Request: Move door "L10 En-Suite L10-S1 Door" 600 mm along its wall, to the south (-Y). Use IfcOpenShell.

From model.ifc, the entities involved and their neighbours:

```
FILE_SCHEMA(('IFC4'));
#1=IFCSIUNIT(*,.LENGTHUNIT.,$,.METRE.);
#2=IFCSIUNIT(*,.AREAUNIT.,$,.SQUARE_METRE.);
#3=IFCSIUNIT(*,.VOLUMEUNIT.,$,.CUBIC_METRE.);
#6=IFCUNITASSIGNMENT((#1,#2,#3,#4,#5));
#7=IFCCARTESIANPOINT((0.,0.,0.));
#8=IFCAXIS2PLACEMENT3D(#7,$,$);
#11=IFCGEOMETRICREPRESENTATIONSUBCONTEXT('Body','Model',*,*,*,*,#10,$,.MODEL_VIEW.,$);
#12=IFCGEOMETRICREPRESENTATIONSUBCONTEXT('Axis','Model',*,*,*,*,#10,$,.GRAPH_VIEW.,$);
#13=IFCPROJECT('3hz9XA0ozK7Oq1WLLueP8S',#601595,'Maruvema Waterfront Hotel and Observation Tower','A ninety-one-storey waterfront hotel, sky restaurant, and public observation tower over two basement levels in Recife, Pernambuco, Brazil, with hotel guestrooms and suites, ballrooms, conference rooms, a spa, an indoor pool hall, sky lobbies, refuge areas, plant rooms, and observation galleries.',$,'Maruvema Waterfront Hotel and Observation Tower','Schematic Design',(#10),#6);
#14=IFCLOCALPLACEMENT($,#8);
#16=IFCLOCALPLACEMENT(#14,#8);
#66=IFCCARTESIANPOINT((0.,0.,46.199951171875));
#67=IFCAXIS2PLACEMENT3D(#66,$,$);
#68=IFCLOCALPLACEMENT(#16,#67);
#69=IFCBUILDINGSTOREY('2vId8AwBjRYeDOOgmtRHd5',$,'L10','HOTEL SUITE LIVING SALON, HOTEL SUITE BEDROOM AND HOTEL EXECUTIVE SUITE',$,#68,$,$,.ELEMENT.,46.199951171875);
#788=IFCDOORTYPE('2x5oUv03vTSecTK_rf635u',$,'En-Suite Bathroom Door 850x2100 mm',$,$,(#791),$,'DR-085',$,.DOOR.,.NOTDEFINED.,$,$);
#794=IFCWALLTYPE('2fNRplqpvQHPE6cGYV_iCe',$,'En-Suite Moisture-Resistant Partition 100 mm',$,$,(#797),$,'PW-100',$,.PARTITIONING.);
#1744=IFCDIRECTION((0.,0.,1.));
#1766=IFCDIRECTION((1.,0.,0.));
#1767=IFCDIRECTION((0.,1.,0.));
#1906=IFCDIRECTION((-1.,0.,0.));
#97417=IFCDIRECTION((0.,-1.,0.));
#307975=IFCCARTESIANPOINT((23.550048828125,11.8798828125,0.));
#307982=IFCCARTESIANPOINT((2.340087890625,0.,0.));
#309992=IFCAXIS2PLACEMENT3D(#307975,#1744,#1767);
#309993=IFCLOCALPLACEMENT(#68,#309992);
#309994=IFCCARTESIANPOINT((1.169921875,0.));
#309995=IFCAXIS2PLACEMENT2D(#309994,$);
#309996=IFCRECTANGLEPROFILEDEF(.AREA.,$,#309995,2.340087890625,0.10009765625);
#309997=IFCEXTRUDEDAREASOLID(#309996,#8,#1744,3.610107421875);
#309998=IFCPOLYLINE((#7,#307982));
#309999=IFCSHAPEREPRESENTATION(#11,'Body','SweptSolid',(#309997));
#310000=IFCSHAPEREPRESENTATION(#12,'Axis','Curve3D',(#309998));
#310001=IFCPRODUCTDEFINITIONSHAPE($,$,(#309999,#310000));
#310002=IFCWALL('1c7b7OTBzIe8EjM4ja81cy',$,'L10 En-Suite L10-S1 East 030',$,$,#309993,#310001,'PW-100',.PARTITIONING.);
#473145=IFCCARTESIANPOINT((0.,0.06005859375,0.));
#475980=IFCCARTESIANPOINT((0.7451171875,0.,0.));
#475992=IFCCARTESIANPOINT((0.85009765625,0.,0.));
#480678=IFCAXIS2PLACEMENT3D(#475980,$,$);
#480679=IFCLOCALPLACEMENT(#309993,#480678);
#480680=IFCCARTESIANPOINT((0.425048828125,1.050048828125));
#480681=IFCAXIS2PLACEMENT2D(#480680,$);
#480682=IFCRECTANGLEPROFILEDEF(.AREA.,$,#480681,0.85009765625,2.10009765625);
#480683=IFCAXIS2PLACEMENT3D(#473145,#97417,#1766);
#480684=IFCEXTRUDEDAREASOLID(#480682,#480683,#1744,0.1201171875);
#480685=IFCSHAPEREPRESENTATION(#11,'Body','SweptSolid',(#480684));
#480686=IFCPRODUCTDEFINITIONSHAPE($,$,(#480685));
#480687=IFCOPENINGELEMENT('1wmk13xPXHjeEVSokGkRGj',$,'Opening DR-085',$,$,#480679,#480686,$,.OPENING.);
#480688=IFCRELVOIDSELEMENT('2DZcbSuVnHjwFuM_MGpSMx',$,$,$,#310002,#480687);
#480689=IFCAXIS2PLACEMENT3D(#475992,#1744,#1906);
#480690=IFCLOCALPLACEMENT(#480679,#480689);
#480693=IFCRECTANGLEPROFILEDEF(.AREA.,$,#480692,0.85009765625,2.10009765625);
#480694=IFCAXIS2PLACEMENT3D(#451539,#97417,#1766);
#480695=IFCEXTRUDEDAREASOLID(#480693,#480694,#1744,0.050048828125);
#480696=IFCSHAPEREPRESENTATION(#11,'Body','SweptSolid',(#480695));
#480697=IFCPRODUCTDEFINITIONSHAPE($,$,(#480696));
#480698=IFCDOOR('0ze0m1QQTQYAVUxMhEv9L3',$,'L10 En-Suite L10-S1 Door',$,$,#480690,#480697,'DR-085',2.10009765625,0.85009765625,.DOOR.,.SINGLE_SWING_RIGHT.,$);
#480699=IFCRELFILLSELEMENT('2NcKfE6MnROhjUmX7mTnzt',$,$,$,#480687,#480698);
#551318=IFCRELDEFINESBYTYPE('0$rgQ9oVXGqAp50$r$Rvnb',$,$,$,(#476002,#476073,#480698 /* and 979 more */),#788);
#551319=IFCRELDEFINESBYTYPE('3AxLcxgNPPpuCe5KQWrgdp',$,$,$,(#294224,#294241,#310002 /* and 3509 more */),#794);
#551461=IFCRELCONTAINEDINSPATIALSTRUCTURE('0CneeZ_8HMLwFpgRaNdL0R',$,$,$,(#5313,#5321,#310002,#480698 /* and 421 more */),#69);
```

```python
import ifcopenshell
import ifcopenshell.api.geometry
import ifcopenshell.util.placement

model = ifcopenshell.open("model.ifc")

door = model.by_guid("0ze0m1QQTQYAVUxMhEv9L3")
opening = door.FillsVoids[0].RelatingOpeningElement
wall = opening.VoidsElements[0].RelatingBuildingElement

wall_matrix = ifcopenshell.util.placement.get_local_placement(wall.ObjectPlacement)
shift = wall_matrix[:3, 0] * -0.6
before = ifcopenshell.util.placement.get_local_placement(door.ObjectPlacement)[:3, 3].copy()

# The door is placed relative to its opening, so it follows when the opening moves.
matrix = ifcopenshell.util.placement.get_local_placement(opening.ObjectPlacement)
matrix[:3, 3] += shift
ifcopenshell.api.geometry.edit_object_placement(
    model, product=opening, matrix=matrix, is_si=False, should_transform_children=True
)

after = ifcopenshell.util.placement.get_local_placement(door.ObjectPlacement)[:3, 3]
print("door moved by", (after - before).round(3) + 0.0)

model.write("model_v2.ifc")
```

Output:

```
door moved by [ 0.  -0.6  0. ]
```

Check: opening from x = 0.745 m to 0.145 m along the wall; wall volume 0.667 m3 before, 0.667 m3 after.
